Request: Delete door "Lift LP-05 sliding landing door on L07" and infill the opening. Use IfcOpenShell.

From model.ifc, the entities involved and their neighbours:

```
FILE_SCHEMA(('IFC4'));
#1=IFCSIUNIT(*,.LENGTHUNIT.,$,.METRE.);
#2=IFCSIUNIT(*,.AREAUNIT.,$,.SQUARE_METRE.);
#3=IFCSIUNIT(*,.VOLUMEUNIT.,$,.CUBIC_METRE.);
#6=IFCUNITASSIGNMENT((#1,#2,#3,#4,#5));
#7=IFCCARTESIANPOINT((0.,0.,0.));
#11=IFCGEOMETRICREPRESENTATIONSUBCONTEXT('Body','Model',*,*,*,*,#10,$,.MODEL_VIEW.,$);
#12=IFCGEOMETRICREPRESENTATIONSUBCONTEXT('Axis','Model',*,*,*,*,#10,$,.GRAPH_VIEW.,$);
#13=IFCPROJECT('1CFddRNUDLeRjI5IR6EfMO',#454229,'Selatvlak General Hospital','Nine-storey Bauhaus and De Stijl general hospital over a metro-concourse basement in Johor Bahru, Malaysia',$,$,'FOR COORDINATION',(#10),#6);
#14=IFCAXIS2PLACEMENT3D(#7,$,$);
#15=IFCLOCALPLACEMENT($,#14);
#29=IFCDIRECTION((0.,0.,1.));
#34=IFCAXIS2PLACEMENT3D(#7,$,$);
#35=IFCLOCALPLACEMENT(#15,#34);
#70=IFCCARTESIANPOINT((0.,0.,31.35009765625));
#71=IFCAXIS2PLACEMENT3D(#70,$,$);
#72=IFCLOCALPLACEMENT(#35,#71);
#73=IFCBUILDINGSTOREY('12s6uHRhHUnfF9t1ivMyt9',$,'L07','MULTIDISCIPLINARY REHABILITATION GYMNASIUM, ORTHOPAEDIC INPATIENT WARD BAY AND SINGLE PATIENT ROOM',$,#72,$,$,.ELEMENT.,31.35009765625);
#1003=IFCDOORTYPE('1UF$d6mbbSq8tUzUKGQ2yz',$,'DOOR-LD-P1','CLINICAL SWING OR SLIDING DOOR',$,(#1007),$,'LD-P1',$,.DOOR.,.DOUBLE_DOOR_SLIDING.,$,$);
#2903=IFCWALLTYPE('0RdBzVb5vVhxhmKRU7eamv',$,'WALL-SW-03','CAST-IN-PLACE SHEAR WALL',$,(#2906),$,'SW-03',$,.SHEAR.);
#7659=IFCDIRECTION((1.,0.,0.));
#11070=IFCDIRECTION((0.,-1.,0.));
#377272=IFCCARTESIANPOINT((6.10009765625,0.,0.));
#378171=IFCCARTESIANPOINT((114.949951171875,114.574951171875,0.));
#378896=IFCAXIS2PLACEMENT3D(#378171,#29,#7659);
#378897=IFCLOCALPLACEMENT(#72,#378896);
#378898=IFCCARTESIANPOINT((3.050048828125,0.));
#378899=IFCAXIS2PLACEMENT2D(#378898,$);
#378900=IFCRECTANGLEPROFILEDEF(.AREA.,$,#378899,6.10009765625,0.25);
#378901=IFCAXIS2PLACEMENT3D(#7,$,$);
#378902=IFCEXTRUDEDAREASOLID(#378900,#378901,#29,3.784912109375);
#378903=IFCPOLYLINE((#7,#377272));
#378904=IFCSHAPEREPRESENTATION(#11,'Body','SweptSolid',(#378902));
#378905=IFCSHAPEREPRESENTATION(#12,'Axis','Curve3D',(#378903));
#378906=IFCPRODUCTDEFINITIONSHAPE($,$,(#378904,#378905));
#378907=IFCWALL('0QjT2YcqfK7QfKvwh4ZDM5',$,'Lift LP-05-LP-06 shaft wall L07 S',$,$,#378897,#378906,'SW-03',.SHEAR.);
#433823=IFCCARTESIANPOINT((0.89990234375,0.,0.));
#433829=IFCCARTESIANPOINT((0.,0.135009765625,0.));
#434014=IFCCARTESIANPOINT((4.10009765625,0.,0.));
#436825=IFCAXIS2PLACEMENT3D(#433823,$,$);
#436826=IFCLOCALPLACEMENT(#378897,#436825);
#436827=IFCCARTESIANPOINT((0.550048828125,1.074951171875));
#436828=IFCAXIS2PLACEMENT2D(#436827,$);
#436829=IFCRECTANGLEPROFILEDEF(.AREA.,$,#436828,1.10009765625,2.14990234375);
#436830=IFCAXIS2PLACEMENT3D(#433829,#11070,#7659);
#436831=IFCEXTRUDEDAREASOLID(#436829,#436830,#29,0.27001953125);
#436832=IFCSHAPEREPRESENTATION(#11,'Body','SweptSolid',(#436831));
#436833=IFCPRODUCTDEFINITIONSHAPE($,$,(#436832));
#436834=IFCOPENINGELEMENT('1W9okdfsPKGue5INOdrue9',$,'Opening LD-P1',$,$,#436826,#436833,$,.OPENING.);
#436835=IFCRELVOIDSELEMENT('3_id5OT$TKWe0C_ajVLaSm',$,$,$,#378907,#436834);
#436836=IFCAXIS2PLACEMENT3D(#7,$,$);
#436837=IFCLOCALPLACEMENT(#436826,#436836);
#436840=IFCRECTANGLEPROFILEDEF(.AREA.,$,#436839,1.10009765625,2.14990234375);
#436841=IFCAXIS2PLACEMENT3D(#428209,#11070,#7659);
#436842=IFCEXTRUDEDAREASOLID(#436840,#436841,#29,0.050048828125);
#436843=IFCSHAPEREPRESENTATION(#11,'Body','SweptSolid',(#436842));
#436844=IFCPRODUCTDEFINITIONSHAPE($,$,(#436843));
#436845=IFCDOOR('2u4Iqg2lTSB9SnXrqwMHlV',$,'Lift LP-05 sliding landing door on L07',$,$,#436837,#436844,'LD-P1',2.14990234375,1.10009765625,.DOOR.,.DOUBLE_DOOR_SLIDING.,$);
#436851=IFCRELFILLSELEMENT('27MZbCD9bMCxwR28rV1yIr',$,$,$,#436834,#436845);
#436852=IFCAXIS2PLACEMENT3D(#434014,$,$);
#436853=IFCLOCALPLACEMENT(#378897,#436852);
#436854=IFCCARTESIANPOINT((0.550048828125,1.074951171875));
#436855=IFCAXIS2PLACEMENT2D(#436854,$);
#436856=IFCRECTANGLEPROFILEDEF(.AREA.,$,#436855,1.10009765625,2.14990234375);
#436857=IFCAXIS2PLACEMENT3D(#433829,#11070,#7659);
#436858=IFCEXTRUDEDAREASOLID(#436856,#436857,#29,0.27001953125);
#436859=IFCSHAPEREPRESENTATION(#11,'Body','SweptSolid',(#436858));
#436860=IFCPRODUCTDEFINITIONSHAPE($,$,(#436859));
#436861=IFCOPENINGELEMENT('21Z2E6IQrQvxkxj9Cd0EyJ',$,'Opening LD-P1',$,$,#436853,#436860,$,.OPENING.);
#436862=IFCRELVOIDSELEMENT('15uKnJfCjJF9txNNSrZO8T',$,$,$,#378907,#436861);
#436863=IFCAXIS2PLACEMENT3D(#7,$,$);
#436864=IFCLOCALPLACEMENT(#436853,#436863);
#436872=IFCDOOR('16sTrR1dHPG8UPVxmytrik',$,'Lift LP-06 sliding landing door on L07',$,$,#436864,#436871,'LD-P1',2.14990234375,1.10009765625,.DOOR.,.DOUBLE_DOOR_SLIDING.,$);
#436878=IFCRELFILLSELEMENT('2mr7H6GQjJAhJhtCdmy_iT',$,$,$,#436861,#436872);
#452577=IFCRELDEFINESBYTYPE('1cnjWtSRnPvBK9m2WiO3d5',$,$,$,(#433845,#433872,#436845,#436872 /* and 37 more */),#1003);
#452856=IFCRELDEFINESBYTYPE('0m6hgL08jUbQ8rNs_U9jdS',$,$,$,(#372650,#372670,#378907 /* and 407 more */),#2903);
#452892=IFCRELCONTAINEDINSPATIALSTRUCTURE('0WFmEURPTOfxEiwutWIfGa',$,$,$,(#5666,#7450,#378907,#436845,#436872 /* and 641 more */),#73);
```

```python
import ifcopenshell
import ifcopenshell.api.feature
import ifcopenshell.api.root
import ifcopenshell.geom
import ifcopenshell.util.shape

model = ifcopenshell.open("model.ifc")
settings = ifcopenshell.geom.settings()


def volume(element):
    """Net volume in cubic metres, openings subtracted."""
    shape = ifcopenshell.geom.create_shape(settings, element)
    return ifcopenshell.util.shape.get_volume(shape.geometry)


door = model.by_guid("2u4Iqg2lTSB9SnXrqwMHlV")
opening = door.FillsVoids[0].RelatingOpeningElement
wall = opening.VoidsElements[0].RelatingBuildingElement
before = volume(wall)

ifcopenshell.api.root.remove_product(model, product=door)
ifcopenshell.api.feature.remove_feature(model, feature=opening)

after = volume(wall)

print(f"wall volume {before:.3f} -> {after:.3f} m3")

model.write("model_updated.ifc")
```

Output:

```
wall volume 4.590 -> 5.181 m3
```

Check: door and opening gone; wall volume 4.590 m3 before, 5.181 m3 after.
